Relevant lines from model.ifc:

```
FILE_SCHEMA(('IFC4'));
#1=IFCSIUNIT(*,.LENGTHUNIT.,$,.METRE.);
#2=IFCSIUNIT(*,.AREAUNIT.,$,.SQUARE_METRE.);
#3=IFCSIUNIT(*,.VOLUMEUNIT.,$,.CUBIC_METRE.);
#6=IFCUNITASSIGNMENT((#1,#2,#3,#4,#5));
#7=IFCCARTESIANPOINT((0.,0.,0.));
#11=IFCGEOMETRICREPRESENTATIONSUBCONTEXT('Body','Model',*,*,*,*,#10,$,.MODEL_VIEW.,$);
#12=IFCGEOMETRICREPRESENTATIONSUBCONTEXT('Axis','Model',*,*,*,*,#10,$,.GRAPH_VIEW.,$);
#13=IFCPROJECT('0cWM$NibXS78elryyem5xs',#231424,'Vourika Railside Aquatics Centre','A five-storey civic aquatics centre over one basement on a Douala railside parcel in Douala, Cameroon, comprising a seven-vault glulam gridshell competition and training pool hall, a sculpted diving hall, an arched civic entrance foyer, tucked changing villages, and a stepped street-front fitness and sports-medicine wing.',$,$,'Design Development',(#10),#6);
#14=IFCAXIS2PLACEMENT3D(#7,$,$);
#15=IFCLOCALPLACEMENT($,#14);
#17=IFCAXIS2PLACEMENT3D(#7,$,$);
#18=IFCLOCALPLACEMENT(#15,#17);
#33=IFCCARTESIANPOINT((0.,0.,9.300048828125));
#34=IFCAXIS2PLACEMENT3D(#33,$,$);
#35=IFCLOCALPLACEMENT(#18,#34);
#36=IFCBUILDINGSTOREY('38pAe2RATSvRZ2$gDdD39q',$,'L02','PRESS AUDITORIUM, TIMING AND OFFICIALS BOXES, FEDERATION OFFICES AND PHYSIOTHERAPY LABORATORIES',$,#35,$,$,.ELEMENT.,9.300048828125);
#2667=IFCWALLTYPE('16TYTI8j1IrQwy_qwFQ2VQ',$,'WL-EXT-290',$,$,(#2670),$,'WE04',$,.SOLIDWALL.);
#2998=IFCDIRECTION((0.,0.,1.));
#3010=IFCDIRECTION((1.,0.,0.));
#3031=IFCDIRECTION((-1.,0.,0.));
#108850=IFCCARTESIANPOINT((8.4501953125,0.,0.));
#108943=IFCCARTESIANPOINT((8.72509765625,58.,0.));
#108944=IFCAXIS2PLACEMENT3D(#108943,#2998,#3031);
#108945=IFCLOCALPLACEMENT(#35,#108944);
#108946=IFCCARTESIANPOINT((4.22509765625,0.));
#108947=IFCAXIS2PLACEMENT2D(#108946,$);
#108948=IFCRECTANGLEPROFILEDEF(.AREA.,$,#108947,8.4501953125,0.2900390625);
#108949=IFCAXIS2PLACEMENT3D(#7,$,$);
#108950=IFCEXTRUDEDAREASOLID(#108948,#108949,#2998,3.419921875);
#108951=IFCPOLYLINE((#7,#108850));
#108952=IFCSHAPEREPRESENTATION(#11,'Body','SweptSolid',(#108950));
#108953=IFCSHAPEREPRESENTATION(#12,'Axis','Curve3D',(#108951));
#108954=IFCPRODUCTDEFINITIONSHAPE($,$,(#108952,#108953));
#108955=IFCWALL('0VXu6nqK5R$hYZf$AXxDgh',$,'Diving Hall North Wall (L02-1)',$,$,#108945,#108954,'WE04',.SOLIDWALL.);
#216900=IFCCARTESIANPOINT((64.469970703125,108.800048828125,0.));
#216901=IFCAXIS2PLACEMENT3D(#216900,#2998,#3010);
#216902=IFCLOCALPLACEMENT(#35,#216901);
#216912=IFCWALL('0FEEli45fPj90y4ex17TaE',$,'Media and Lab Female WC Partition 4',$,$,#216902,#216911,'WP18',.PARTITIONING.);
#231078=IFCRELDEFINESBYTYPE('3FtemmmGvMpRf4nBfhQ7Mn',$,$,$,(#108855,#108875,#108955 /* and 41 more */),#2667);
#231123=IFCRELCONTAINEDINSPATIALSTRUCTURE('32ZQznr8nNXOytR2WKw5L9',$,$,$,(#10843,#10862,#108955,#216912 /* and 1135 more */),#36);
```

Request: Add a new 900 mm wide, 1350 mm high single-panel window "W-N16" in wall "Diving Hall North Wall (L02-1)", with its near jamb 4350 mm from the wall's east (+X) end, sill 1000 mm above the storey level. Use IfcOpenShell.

```python
import numpy as np
import ifcopenshell
import ifcopenshell.api.feature
import ifcopenshell.api.geometry
import ifcopenshell.api.root
import ifcopenshell.api.spatial
import ifcopenshell.geom
import ifcopenshell.util.element
import ifcopenshell.util.placement
import ifcopenshell.util.representation
import ifcopenshell.util.shape
import ifcopenshell.util.unit

model = ifcopenshell.open("model.ifc")
unit_scale = ifcopenshell.util.unit.calculate_unit_scale(model)
settings = ifcopenshell.geom.settings()


def volume(element):
    """Net volume in cubic metres, openings subtracted."""
    shape = ifcopenshell.geom.create_shape(settings, element)
    return ifcopenshell.util.shape.get_volume(shape.geometry)


wall = model.by_guid("0VXu6nqK5R$hYZf$AXxDgh")
storey = ifcopenshell.util.element.get_container(wall, ifc_class="IfcBuildingStorey")
context = ifcopenshell.util.representation.get_context(model, "Model", "Body", "MODEL_VIEW")
before = volume(wall)

width, height, from_end, sill = 0.9, 1.35, 4.35, 1  # metres

# The wall runs along its own X axis, and the end named is its -X end.
wall_shape = ifcopenshell.geom.create_shape(settings, wall)
x, y, z = ifcopenshell.util.shape.get_vertices(wall_shape.geometry).T
start = x.min() + from_end
face, thickness = float(y.min()), float(y.max() - y.min())
wall_matrix = ifcopenshell.util.placement.get_local_placement(wall.ObjectPlacement)
level = ifcopenshell.util.placement.get_local_placement(storey.ObjectPlacement)[2, 3]


def in_wall(x, y):
    """Placement at x, y metres in the wall's axes, at sill height."""
    matrix = wall_matrix.copy()
    matrix[:, 3] = wall_matrix @ np.array([x / unit_scale, y / unit_scale, 0.0, 1.0])
    matrix[2, 3] = level + sill / unit_scale
    return matrix


# Opening: a box that overshoots both wall faces by 50 mm.
opening = ifcopenshell.api.root.create_entity(model, ifc_class="IfcOpeningElement", predefined_type="OPENING")
box = ifcopenshell.api.geometry.add_wall_representation(
    model, context=context, length=width, height=height, thickness=thickness + 0.1
)
ifcopenshell.api.geometry.assign_representation(model, product=opening, representation=box)
ifcopenshell.api.geometry.edit_object_placement(model, product=opening, matrix=in_wall(start, face - 0.05), is_si=False)
ifcopenshell.api.feature.add_feature(model, feature=opening, element=wall)

window = ifcopenshell.api.root.create_entity(model, ifc_class="IfcWindow", name="W-N16", predefined_type="WINDOW")
window.OverallWidth, window.OverallHeight = width / unit_scale, height / unit_scale
window.PartitioningType = "SINGLE_PANEL"
body = ifcopenshell.api.geometry.add_window_representation(
    model,
    context=context,
    overall_width=window.OverallWidth,
    overall_height=window.OverallHeight,
    partition_type="SINGLE_PANEL",
)
ifcopenshell.api.geometry.assign_representation(model, product=window, representation=body)
ifcopenshell.api.spatial.assign_container(model, products=[window], relating_structure=storey)
ifcopenshell.api.feature.add_filling(model, opening=opening, element=window)

# Centre the window in the wall's thickness.
ifcopenshell.api.geometry.edit_object_placement(model, product=window, matrix=in_wall(start, face), is_si=False)
window_shape = ifcopenshell.geom.create_shape(settings, window)
depth = ifcopenshell.util.shape.get_vertices(window_shape.geometry)[:, 1]
offset = face + thickness / 2 - (depth.min() + depth.max()) / 2
ifcopenshell.api.geometry.edit_object_placement(model, product=window, matrix=in_wall(start, offset), is_si=False)

after = volume(wall)

print(f"wall volume {before:.3f} -> {after:.3f} m3")

model.write("model-out.ifc")
```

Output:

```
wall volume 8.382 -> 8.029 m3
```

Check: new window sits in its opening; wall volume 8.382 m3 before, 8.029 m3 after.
